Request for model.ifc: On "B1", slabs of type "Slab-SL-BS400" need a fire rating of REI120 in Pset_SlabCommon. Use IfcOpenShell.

First a look at what the model holds.

```python
import ifcopenshell
import ifcopenshell.util.element

model = ifcopenshell.open("model.ifc")
print(model.schema)
storey = next(s for s in model.by_type("IfcBuildingStorey") if s.Name == "B1")
slabs = [e for e in ifcopenshell.util.element.get_decomposition(storey) if e.is_a("IfcSlab")]
seen = {}
for e in slabs:
    element_type = ifcopenshell.util.element.get_type(e)
    key = (element_type.Name if element_type != e and element_type else None, ifcopenshell.util.element.get_pset(e, "Pset_SlabCommon", "FireRating"))
    seen[key] = seen.get(key, 0) + 1
for (name, value), count in sorted(seen.items(), key=str):
    print(count, "x", name, "|", value)
```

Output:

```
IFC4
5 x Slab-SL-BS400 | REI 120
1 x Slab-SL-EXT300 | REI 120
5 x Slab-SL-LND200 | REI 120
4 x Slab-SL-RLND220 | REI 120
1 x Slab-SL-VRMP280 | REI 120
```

```python
import ifcopenshell
import ifcopenshell.api.pset
import ifcopenshell.util.element

model = ifcopenshell.open("model.ifc")

storey = next(s for s in model.by_type("IfcBuildingStorey") if s.Name == "B1")
slabs = [e for e in ifcopenshell.util.element.get_decomposition(storey) if e.is_a("IfcSlab")]

count = 0
for e in slabs:
    element_type = ifcopenshell.util.element.get_type(e)
    if element_type in (None, e) or element_type.Name != "Slab-SL-BS400":
        continue
    # add_pset returns the element's existing set when there is one.
    pset = ifcopenshell.api.pset.add_pset(model, product=e, name="Pset_SlabCommon")
    ifcopenshell.api.pset.edit_pset(model, pset=pset, properties={"FireRating": "REI120"})
    count += 1

print(count, "slabs updated")

model.write("model_edited.ifc")
```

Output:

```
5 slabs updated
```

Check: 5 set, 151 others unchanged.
